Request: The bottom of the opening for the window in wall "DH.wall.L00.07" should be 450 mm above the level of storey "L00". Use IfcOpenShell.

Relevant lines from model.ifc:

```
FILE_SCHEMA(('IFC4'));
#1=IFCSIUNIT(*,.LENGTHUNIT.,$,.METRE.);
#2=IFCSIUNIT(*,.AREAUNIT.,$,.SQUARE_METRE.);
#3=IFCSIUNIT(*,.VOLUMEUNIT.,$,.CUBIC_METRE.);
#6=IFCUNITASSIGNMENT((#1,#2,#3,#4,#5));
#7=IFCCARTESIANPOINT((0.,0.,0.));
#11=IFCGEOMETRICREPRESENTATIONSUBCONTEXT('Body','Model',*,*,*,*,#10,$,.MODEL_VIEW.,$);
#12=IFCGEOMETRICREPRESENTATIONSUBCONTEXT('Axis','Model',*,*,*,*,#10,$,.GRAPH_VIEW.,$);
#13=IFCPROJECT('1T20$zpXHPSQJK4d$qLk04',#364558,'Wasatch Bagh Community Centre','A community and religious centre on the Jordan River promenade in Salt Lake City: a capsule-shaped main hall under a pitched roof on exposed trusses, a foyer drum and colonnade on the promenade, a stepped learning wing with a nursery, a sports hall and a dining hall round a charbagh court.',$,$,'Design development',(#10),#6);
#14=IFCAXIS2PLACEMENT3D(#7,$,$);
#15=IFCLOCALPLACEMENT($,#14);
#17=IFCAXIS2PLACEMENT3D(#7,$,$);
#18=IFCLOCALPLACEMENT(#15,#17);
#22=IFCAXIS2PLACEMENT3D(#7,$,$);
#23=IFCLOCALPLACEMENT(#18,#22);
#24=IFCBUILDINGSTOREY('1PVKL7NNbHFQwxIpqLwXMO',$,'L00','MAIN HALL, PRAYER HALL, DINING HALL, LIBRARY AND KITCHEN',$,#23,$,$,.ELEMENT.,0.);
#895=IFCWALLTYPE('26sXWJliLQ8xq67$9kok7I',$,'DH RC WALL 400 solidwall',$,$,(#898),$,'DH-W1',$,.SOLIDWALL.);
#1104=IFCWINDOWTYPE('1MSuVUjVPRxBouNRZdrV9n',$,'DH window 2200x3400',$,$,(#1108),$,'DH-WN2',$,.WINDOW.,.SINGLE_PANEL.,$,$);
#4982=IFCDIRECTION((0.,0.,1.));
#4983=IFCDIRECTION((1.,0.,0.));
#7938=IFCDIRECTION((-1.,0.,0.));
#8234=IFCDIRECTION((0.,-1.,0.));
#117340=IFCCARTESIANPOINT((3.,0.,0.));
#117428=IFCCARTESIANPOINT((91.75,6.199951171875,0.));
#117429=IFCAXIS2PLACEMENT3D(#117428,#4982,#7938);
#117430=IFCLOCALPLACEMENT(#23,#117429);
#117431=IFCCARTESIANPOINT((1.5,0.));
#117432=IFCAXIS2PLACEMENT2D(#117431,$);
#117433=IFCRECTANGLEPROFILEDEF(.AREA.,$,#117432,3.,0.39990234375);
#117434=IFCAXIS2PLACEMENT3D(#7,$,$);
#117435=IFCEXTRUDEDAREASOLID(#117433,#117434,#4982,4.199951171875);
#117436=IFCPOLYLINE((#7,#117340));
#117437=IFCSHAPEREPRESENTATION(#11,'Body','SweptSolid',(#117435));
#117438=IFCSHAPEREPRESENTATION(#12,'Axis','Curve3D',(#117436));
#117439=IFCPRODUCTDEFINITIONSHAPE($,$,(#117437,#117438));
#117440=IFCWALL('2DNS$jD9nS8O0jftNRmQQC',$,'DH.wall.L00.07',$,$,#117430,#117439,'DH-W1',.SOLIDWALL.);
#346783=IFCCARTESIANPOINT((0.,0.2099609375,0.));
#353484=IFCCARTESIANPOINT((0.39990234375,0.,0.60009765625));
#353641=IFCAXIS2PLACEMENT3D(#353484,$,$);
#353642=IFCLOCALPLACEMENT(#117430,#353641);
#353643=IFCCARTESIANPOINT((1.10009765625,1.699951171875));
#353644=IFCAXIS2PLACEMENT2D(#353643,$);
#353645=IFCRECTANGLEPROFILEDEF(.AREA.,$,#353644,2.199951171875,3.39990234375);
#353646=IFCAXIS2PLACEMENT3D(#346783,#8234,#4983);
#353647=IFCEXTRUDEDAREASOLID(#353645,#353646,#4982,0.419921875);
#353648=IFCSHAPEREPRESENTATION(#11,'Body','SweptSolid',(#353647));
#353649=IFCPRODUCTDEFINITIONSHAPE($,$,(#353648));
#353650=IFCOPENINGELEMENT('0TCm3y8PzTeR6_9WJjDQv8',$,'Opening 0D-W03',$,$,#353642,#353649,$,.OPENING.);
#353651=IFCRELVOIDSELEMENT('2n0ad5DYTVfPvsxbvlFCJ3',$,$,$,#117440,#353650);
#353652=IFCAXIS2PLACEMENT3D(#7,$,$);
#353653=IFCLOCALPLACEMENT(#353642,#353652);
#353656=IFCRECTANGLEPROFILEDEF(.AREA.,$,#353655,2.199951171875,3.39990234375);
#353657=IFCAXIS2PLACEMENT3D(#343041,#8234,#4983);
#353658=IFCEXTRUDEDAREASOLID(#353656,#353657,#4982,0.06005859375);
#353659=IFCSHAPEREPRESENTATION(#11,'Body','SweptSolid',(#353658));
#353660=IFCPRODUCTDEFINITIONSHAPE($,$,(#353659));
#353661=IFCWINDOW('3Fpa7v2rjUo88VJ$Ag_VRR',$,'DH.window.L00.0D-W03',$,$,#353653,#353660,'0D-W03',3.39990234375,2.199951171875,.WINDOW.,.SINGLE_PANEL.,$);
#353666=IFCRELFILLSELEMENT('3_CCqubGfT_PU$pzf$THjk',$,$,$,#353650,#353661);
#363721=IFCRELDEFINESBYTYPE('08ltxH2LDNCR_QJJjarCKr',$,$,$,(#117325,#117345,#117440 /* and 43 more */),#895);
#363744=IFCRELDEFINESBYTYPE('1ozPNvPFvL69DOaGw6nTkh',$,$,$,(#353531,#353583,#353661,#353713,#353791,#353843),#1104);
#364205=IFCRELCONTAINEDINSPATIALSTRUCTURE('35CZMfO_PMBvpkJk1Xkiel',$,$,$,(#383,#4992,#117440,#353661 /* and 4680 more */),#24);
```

```python
import numpy as np
import ifcopenshell
import ifcopenshell.api.geometry
import ifcopenshell.geom
import ifcopenshell.util.element
import ifcopenshell.util.placement
import ifcopenshell.util.shape
import ifcopenshell.util.unit

model = ifcopenshell.open("model.ifc")
unit_scale = ifcopenshell.util.unit.calculate_unit_scale(model)

window = model.by_guid("3Fpa7v2rjUo88VJ$Ag_VRR")
opening = window.FillsVoids[0].RelatingOpeningElement
storey = ifcopenshell.util.element.get_container(window, ifc_class="IfcBuildingStorey")
level = ifcopenshell.util.placement.get_local_placement(storey.ObjectPlacement)[2, 3]

# The opening's origin need not be at the sill, so measure its lowest point.
shape = ifcopenshell.geom.create_shape(ifcopenshell.geom.settings(), opening)
bottom = ifcopenshell.util.shape.get_shape_bottom_elevation(shape, shape.geometry) / unit_scale
dz = level + 0.45 - bottom

shift = np.array([0.0, 0.0, dz])
# The window is placed relative to its opening, so it follows when the opening moves.
matrix = ifcopenshell.util.placement.get_local_placement(opening.ObjectPlacement)
matrix[:3, 3] += shift
ifcopenshell.api.geometry.edit_object_placement(
    model, product=opening, matrix=matrix, is_si=False, should_transform_children=True
)

print(f"moved by {dz * unit_scale:+.3f} m")

model.write("model_edited.ifc")
```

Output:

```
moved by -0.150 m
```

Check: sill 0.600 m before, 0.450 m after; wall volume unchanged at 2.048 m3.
